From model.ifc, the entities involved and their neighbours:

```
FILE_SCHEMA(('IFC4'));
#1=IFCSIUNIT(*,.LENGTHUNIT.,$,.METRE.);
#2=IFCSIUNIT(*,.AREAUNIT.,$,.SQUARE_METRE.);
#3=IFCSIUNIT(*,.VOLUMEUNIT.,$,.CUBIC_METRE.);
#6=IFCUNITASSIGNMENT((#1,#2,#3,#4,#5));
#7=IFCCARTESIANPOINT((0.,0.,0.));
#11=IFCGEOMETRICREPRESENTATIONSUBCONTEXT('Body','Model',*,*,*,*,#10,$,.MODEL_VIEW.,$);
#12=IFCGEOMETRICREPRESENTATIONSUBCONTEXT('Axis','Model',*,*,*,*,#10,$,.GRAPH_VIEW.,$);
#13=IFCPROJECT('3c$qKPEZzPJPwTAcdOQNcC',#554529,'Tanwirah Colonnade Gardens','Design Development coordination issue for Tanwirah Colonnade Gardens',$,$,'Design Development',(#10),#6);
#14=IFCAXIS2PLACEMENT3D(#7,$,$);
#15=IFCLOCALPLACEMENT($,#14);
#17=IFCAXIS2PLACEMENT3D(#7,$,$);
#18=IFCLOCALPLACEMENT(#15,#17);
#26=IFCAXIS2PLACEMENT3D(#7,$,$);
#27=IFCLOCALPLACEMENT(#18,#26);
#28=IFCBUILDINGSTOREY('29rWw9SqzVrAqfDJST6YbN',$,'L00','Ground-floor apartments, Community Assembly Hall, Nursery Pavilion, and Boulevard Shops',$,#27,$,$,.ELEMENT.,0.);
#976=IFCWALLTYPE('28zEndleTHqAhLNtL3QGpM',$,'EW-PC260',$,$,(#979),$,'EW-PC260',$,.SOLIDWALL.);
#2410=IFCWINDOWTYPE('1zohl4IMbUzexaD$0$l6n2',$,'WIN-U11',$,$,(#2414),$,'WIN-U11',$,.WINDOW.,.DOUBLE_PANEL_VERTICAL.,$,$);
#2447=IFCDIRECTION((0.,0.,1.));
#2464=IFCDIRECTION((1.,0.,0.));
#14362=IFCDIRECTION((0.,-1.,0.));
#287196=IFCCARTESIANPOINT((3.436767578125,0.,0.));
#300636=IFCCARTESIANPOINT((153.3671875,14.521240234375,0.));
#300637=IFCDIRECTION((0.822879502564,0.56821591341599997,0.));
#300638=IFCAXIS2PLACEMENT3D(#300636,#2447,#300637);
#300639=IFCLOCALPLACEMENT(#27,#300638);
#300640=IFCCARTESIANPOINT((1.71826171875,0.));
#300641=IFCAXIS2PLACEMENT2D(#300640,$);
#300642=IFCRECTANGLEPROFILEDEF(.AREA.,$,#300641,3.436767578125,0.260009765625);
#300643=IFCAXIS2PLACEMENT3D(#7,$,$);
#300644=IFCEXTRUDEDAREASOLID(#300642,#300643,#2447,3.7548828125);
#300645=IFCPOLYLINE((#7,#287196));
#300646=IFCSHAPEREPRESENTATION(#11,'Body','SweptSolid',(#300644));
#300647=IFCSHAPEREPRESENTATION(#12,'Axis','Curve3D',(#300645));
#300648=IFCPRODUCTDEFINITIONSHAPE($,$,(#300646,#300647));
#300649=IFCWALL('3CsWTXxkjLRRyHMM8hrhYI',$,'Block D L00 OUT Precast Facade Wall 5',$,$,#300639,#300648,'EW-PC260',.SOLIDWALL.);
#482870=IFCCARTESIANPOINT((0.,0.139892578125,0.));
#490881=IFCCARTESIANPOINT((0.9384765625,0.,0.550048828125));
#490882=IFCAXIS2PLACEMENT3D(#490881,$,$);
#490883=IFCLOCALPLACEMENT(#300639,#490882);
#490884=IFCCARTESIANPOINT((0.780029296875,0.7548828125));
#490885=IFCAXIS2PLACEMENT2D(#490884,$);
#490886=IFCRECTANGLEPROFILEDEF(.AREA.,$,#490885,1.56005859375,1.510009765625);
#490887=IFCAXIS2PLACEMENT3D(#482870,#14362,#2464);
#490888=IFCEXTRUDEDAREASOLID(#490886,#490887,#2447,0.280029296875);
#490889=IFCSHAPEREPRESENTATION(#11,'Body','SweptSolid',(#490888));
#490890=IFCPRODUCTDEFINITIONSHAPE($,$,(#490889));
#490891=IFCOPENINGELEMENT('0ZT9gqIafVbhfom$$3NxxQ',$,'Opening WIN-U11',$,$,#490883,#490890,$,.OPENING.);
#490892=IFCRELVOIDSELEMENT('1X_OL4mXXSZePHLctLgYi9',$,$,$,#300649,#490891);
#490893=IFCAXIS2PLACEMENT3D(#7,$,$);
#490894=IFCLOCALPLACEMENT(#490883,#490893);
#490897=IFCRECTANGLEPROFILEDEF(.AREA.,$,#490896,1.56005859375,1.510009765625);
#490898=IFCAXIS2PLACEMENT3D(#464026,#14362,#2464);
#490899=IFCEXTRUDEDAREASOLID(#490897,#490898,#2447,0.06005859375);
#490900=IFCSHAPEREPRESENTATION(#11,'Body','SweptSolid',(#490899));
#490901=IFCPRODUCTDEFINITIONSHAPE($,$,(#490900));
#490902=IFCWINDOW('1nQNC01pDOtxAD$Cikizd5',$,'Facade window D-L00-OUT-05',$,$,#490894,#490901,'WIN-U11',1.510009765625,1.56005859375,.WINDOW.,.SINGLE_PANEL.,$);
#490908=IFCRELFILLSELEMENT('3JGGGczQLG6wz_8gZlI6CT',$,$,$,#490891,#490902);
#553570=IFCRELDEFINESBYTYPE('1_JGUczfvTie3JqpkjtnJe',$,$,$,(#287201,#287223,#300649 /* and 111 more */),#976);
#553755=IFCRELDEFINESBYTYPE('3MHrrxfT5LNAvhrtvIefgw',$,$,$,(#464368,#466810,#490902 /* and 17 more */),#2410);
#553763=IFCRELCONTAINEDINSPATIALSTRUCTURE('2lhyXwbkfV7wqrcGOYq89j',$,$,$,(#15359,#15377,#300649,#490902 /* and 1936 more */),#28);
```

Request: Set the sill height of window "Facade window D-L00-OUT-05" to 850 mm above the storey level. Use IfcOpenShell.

```python
import numpy as np
import ifcopenshell
import ifcopenshell.api.geometry
import ifcopenshell.geom
import ifcopenshell.util.element
import ifcopenshell.util.placement
import ifcopenshell.util.shape
import ifcopenshell.util.unit

model = ifcopenshell.open("model.ifc")
unit_scale = ifcopenshell.util.unit.calculate_unit_scale(model)

window = model.by_guid("1nQNC01pDOtxAD$Cikizd5")
opening = window.FillsVoids[0].RelatingOpeningElement
storey = ifcopenshell.util.element.get_container(window, ifc_class="IfcBuildingStorey")
level = ifcopenshell.util.placement.get_local_placement(storey.ObjectPlacement)[2, 3]

# The opening's origin need not be at the sill, so measure its lowest point.
shape = ifcopenshell.geom.create_shape(ifcopenshell.geom.settings(), opening)
bottom = ifcopenshell.util.shape.get_shape_bottom_elevation(shape, shape.geometry) / unit_scale
dz = level + 0.85 - bottom

shift = np.array([0.0, 0.0, dz])
# The window is placed relative to its opening, so it follows when the opening moves.
matrix = ifcopenshell.util.placement.get_local_placement(opening.ObjectPlacement)
matrix[:3, 3] += shift
ifcopenshell.api.geometry.edit_object_placement(
    model, product=opening, matrix=matrix, is_si=False, should_transform_children=True
)

print(f"moved by {dz * unit_scale:+.3f} m")

model.write("model_edited.ifc")
```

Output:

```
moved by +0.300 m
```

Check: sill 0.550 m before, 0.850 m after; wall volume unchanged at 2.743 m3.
